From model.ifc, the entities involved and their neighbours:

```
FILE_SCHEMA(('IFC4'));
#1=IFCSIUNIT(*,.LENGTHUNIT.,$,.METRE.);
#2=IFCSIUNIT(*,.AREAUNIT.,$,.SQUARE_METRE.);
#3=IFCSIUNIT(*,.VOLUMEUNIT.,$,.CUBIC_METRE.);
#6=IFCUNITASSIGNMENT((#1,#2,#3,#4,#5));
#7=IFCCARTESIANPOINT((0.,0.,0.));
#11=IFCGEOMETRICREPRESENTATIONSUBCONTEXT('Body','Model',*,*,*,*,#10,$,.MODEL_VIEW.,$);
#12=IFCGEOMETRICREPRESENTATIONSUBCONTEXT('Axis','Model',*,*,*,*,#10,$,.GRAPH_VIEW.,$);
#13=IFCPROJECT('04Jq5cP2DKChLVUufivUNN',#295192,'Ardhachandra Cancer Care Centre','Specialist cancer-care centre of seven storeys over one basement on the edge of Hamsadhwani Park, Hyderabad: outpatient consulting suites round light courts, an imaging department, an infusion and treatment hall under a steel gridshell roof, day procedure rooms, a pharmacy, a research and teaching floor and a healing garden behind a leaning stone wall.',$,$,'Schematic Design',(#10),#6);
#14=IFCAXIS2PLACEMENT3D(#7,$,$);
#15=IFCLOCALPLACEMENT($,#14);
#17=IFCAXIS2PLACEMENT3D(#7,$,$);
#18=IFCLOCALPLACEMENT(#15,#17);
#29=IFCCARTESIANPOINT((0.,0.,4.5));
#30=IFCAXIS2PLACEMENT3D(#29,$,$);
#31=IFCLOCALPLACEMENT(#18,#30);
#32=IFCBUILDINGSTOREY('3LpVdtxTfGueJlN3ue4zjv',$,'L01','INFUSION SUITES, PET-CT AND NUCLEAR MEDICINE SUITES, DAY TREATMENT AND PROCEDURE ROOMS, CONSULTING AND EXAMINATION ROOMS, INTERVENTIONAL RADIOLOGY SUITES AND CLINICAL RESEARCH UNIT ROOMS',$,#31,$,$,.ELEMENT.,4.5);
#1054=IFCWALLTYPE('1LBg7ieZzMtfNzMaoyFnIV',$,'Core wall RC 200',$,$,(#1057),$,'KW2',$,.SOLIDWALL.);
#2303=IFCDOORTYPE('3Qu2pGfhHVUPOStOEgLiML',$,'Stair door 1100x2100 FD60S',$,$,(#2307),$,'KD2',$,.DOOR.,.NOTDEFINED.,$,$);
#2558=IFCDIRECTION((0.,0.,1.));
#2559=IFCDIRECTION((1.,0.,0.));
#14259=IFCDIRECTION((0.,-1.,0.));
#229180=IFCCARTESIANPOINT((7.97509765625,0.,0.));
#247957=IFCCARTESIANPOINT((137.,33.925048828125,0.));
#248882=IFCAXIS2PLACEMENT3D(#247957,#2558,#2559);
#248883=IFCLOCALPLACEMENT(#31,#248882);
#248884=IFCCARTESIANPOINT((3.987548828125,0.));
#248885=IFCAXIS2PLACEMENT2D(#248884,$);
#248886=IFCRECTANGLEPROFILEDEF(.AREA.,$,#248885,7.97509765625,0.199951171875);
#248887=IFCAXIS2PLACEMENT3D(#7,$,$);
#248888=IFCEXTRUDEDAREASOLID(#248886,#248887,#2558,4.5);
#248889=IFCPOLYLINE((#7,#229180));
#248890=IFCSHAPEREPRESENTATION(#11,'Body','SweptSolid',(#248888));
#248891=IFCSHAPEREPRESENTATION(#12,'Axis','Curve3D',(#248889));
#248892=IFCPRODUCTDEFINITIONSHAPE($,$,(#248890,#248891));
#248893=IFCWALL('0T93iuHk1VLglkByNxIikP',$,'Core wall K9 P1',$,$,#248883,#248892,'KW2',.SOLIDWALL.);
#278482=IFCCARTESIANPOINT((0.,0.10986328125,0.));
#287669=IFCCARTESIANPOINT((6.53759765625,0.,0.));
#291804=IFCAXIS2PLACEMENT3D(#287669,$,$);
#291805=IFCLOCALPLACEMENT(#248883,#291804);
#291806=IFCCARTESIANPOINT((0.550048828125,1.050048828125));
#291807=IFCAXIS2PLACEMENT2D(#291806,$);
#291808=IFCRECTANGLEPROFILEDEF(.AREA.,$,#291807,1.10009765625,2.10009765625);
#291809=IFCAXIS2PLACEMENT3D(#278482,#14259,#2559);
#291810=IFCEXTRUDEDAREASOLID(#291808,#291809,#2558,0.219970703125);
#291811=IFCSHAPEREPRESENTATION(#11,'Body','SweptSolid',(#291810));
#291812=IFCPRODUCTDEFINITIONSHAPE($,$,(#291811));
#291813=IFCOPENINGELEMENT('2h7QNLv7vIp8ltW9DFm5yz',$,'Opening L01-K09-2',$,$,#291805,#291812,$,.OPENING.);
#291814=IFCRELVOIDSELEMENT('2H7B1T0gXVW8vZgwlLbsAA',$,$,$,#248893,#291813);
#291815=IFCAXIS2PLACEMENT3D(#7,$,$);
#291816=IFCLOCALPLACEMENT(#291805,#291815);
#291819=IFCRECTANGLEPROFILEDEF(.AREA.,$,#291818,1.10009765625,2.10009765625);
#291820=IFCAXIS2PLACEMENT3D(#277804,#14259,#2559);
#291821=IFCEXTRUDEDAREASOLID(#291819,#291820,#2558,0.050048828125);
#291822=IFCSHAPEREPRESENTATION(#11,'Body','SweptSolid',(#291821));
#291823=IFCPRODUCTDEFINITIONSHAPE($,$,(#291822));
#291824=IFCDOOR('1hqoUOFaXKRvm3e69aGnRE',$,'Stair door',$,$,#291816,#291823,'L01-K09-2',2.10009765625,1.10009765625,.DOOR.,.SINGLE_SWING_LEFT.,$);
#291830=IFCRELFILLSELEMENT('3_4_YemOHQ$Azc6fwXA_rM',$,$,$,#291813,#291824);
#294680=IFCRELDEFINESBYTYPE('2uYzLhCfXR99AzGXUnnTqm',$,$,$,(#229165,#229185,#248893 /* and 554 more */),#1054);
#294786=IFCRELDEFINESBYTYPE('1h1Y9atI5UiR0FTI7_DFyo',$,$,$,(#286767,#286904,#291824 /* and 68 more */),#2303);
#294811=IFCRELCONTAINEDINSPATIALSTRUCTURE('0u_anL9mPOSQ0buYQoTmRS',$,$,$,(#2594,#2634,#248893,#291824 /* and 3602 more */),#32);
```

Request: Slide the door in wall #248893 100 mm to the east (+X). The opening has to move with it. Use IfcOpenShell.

```python
import ifcopenshell
import ifcopenshell.api.geometry
import ifcopenshell.util.placement

model = ifcopenshell.open("model.ifc")

door = model.by_guid("1hqoUOFaXKRvm3e69aGnRE")
opening = door.FillsVoids[0].RelatingOpeningElement
wall = opening.VoidsElements[0].RelatingBuildingElement

wall_matrix = ifcopenshell.util.placement.get_local_placement(wall.ObjectPlacement)
shift = wall_matrix[:3, 0] * 0.1
before = ifcopenshell.util.placement.get_local_placement(door.ObjectPlacement)[:3, 3].copy()

# The door is placed relative to its opening, so it follows when the opening moves.
matrix = ifcopenshell.util.placement.get_local_placement(opening.ObjectPlacement)
matrix[:3, 3] += shift
ifcopenshell.api.geometry.edit_object_placement(
    model, product=opening, matrix=matrix, is_si=False, should_transform_children=True
)

after = ifcopenshell.util.placement.get_local_placement(door.ObjectPlacement)[:3, 3]
print("door moved by", (after - before).round(3) + 0.0)

model.write("model_rev.ifc")
```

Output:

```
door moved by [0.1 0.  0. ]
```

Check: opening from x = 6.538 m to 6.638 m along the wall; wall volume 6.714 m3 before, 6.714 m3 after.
